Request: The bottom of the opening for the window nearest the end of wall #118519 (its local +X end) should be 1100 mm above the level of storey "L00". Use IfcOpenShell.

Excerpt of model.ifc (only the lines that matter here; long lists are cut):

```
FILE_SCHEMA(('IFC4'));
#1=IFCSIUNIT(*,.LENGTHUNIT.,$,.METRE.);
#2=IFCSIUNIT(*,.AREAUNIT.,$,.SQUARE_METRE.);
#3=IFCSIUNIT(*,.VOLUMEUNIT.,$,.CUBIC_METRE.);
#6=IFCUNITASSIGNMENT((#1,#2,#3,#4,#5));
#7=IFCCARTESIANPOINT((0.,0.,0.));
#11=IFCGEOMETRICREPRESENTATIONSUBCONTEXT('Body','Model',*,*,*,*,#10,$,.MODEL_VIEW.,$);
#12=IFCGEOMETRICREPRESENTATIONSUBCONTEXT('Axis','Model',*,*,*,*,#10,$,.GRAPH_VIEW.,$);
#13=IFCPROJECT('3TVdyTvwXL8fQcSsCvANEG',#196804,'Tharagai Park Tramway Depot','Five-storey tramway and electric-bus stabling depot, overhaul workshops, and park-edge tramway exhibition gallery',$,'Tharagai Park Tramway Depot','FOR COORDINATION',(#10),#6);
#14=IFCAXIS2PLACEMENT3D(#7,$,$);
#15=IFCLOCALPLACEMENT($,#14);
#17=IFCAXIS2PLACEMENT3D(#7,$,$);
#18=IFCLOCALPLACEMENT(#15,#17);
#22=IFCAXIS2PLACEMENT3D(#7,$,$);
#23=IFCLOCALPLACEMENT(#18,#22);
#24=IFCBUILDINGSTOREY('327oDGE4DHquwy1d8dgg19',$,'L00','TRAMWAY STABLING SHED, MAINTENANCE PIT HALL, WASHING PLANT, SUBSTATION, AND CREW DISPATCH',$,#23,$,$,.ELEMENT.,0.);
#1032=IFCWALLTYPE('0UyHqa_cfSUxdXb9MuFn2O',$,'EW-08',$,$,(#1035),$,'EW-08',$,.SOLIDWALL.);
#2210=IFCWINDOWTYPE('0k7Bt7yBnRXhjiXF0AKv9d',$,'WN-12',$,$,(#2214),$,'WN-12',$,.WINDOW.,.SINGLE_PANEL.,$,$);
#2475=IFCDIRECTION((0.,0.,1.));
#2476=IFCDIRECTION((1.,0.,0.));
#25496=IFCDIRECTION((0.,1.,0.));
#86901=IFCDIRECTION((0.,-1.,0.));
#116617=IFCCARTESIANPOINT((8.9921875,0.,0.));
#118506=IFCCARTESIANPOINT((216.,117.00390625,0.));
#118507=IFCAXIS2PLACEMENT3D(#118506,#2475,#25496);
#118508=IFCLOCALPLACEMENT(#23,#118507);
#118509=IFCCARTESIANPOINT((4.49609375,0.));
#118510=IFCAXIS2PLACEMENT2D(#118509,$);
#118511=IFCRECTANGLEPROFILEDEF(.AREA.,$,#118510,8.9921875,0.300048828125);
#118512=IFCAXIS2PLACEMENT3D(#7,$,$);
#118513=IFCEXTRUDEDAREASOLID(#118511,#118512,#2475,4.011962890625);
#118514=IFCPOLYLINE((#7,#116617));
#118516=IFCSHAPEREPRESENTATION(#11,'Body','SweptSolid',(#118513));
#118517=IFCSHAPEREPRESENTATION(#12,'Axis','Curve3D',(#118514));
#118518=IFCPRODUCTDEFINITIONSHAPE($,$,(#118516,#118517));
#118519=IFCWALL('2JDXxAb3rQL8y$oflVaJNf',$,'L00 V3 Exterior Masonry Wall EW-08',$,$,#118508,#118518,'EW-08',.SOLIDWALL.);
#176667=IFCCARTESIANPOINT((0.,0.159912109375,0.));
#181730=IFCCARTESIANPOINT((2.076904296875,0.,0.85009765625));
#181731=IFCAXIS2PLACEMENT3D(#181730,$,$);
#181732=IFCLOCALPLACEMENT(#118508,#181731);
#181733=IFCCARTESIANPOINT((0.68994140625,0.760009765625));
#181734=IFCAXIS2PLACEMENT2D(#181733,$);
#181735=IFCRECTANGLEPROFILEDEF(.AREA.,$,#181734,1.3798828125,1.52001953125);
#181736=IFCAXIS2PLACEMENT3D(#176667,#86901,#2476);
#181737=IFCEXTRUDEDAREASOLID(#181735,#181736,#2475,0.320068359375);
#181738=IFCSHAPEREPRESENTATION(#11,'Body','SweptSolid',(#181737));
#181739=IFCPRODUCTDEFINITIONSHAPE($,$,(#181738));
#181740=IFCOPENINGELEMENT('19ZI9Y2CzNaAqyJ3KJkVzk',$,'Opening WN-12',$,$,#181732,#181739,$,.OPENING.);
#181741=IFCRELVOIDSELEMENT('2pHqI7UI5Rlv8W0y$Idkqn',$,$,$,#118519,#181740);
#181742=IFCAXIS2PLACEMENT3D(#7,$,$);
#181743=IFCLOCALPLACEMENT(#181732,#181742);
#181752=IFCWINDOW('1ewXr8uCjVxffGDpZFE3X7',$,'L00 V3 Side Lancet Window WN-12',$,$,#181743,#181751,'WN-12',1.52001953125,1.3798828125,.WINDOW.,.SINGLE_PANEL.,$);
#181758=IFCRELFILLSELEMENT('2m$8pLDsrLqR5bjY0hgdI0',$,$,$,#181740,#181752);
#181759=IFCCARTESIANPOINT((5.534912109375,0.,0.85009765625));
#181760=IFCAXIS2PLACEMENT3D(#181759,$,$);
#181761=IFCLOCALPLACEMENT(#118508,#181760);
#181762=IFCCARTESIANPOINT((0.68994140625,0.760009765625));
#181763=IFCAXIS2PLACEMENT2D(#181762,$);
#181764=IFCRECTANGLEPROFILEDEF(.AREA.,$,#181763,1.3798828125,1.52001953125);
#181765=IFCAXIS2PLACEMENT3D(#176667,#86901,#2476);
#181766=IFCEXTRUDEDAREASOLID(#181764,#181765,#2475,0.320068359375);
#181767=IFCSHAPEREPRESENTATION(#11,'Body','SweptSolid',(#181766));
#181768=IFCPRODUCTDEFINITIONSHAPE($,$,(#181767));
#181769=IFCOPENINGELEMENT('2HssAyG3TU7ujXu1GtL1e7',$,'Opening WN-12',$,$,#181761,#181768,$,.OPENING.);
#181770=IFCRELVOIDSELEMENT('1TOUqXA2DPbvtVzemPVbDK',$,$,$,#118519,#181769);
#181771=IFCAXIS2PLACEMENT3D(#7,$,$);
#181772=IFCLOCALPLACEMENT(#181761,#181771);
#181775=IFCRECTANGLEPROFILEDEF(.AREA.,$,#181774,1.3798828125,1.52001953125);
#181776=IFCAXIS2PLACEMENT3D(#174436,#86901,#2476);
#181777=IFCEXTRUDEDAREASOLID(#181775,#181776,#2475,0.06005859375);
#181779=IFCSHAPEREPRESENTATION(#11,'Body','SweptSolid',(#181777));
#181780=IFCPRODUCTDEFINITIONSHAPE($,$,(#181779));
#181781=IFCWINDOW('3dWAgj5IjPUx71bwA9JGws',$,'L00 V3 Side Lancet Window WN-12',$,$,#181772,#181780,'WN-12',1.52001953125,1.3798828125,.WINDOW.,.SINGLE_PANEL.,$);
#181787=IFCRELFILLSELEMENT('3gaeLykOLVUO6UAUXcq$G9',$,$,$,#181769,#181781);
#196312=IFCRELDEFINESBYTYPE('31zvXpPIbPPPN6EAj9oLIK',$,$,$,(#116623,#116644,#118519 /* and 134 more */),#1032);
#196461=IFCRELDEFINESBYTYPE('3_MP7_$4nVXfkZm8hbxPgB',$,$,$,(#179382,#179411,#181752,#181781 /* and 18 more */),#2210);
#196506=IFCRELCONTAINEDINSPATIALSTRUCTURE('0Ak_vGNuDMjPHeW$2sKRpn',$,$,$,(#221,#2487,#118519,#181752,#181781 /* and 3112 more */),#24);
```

```python
import numpy as np
import ifcopenshell
import ifcopenshell.api.geometry
import ifcopenshell.geom
import ifcopenshell.util.element
import ifcopenshell.util.placement
import ifcopenshell.util.shape
import ifcopenshell.util.unit

model = ifcopenshell.open("model.ifc")
unit_scale = ifcopenshell.util.unit.calculate_unit_scale(model)

window = model.by_guid("3dWAgj5IjPUx71bwA9JGws")
opening = window.FillsVoids[0].RelatingOpeningElement
storey = ifcopenshell.util.element.get_container(window, ifc_class="IfcBuildingStorey")
level = ifcopenshell.util.placement.get_local_placement(storey.ObjectPlacement)[2, 3]

# The opening's origin need not be at the sill, so measure its lowest point.
shape = ifcopenshell.geom.create_shape(ifcopenshell.geom.settings(), opening)
bottom = ifcopenshell.util.shape.get_shape_bottom_elevation(shape, shape.geometry) / unit_scale
dz = level + 1.1 / unit_scale - bottom

shift = np.array([0.0, 0.0, dz])
# The window is placed relative to its opening, so it follows when the opening moves.
matrix = ifcopenshell.util.placement.get_local_placement(opening.ObjectPlacement)
matrix[:3, 3] += shift
ifcopenshell.api.geometry.edit_object_placement(
    model, product=opening, matrix=matrix, is_si=False, should_transform_children=True
)

print(f"moved by {dz * unit_scale:+.3f} m")

model.write("model-out.ifc")
```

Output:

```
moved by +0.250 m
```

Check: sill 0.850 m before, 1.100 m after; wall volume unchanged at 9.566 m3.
